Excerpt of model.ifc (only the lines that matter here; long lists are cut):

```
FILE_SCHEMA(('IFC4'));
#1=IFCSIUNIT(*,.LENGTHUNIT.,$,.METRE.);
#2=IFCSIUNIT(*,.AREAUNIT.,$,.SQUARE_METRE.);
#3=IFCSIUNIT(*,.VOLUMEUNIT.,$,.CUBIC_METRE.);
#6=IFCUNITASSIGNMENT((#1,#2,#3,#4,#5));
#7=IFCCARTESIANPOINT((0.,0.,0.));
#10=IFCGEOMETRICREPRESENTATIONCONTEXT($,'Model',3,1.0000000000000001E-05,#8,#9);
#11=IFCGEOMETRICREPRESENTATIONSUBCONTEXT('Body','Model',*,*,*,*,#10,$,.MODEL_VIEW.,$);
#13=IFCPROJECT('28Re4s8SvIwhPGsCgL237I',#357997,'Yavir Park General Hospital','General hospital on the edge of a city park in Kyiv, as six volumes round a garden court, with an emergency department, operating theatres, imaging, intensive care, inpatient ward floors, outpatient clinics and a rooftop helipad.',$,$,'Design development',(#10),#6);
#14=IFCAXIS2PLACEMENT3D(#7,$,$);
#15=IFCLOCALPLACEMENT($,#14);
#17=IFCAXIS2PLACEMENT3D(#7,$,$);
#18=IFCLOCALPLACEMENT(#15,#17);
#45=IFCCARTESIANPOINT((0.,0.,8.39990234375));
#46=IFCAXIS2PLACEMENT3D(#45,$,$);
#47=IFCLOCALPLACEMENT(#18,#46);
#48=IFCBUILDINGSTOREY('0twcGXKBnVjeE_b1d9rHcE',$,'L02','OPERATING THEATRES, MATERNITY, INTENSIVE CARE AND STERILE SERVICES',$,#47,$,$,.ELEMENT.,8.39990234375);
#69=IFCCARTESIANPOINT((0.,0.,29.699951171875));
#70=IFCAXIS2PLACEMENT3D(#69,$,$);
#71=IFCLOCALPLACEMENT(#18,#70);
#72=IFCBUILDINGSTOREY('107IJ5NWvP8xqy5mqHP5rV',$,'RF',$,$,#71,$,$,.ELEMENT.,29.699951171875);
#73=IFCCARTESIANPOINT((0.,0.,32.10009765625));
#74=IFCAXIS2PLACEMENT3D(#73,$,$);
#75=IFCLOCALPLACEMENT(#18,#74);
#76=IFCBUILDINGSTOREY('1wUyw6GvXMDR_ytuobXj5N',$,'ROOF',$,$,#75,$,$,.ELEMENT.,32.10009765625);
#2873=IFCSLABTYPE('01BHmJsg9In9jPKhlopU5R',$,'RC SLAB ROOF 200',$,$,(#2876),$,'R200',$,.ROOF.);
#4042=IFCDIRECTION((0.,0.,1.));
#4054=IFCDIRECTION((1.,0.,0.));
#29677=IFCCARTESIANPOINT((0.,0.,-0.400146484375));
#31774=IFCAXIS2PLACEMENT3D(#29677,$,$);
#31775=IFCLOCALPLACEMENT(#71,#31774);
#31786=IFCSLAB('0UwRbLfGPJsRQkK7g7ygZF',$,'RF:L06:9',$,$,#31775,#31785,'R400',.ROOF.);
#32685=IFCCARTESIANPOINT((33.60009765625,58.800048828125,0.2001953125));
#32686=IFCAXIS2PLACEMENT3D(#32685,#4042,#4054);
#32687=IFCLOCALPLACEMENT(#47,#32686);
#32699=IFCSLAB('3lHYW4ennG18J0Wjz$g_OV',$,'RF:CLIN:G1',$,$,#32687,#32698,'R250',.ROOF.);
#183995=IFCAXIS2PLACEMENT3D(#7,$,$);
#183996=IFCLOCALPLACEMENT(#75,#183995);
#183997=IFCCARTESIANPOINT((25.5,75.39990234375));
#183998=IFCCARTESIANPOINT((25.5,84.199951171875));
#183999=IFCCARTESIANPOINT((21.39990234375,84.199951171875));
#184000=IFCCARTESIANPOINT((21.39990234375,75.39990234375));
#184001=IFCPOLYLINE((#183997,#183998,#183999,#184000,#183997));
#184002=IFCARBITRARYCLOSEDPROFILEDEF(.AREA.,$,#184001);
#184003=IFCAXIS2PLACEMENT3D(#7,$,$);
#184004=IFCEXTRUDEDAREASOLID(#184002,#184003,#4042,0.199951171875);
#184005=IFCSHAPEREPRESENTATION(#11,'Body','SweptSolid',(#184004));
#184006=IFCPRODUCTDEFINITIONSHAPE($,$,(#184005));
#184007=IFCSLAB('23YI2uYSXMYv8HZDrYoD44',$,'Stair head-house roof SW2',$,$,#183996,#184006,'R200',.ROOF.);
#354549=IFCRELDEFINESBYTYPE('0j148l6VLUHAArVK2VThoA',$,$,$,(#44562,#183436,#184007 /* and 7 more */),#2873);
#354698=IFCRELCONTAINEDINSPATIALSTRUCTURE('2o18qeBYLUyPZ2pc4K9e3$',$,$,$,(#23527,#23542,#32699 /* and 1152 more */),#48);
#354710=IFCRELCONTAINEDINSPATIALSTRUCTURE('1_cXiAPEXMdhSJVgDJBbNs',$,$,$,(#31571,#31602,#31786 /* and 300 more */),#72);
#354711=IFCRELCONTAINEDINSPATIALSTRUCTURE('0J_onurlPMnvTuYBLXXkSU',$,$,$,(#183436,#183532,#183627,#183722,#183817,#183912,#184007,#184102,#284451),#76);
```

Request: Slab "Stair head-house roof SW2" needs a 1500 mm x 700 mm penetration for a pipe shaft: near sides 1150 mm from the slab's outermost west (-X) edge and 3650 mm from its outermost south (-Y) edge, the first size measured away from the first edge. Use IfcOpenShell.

```python
import numpy as np
import ifcopenshell
import ifcopenshell.api.feature
import ifcopenshell.api.geometry
import ifcopenshell.api.root
import ifcopenshell.geom
import ifcopenshell.util.placement
import ifcopenshell.util.representation
import ifcopenshell.util.shape
import ifcopenshell.util.unit

model = ifcopenshell.open("model.ifc")
unit_scale = ifcopenshell.util.unit.calculate_unit_scale(model)
settings = ifcopenshell.geom.settings()


def volume(element):
    """Net volume in cubic metres, openings subtracted."""
    shape = ifcopenshell.geom.create_shape(settings, element)
    return ifcopenshell.util.shape.get_volume(shape.geometry)


slab = model.by_guid("23YI2uYSXMYv8HZDrYoD44")
before = volume(slab)

# Extent in the slab's own axes, in metres. The edges named are its -X and -Y sides.
slab_shape = ifcopenshell.geom.create_shape(settings, slab)
vertices = ifcopenshell.util.shape.get_vertices(slab_shape.geometry)
x_min, y_min, bottom = vertices.min(axis=0)
top = vertices[:, 2].max()

opening = ifcopenshell.api.root.create_entity(model, ifc_class="IfcOpeningElement", name="Pipe shaft opening", predefined_type="OPENING")
context = ifcopenshell.util.representation.get_context(model, "Model", "Body", "MODEL_VIEW")
width, depth = 1.5, 0.7
outline = [(0.0, 0.0), (width, 0.0), (width, depth), (0.0, depth), (0.0, 0.0)]
# Overshoot both faces by 50 mm so the cut is clean.
shape = ifcopenshell.api.geometry.add_slab_representation(
    model, context=context, depth=top - bottom + 0.1, polyline=outline
)
ifcopenshell.api.geometry.assign_representation(model, product=opening, representation=shape)

matrix = ifcopenshell.util.placement.get_local_placement(slab.ObjectPlacement)
matrix[:, 3] = matrix @ np.append(np.array([x_min + 1.15, y_min + 3.65, bottom - 0.05]) / unit_scale, 1.0)
ifcopenshell.api.geometry.edit_object_placement(model, product=opening, matrix=matrix, is_si=False)
ifcopenshell.api.feature.add_feature(model, feature=opening, element=slab)

after = volume(slab)

print(f"slab volume {before:.3f} -> {after:.3f} m3")

model.write("model_edited.ifc")
```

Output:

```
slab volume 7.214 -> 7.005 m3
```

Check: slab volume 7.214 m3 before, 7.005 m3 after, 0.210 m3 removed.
